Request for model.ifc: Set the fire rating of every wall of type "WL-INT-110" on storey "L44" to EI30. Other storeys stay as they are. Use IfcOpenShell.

First a look at what the model holds.

```python
import ifcopenshell
import ifcopenshell.util.element

model = ifcopenshell.open("model.ifc")
print(model.schema)
storey = next(s for s in model.by_type("IfcBuildingStorey") if s.Name == "L44")
walls = [e for e in ifcopenshell.util.element.get_decomposition(storey) if e.is_a("IfcWall")]
seen = {}
for e in walls:
    element_type = ifcopenshell.util.element.get_type(e)
    key = (element_type.Name if element_type != e and element_type else None, ifcopenshell.util.element.get_pset(e, "Pset_WallCommon", "FireRating"))
    seen[key] = seen.get(key, 0) + 1
for (name, value), count in sorted(seen.items(), key=str):
    print(count, "x", name, "|", value)
```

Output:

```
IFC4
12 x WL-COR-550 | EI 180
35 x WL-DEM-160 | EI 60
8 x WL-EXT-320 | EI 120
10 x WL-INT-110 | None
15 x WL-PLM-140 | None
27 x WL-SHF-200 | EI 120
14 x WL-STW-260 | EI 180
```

```python
import ifcopenshell
import ifcopenshell.api.pset
import ifcopenshell.util.element

model = ifcopenshell.open("model.ifc")

storey = next(s for s in model.by_type("IfcBuildingStorey") if s.Name == "L44")
walls = [e for e in ifcopenshell.util.element.get_decomposition(storey) if e.is_a("IfcWall")]

count = 0
for e in walls:
    element_type = ifcopenshell.util.element.get_type(e)
    if element_type in (None, e) or element_type.Name != "WL-INT-110":
        continue
    found = ifcopenshell.util.element.get_pset(e, "Pset_WallCommon", should_inherit=False)
    if found:
        pset = model.by_id(found["id"])
        if len(ifcopenshell.util.element.get_elements_by_pset(pset)) > 1:
            pset = ifcopenshell.api.pset.unshare_pset(model, products=[e], pset=pset)[0]
    else:
        pset = ifcopenshell.api.pset.add_pset(model, product=e, name="Pset_WallCommon")
    ifcopenshell.api.pset.edit_pset(model, pset=pset, properties={"FireRating": "EI30"})
    count += 1

print(count, "walls updated")

model.write("model-out.ifc")
```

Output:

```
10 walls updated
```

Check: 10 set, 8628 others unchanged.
